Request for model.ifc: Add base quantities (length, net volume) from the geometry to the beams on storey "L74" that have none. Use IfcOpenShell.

First a look at what the model holds.

```python
import ifcopenshell
import ifcopenshell.util.element
import ifcopenshell.util.unit

model = ifcopenshell.open("model.ifc")
print(model.schema)
for unit_type in ("LENGTHUNIT", "AREAUNIT", "VOLUMEUNIT"):
    print(unit_type, ifcopenshell.util.unit.calculate_unit_scale(model, unit_type))
storey = next(s for s in model.by_type("IfcBuildingStorey") if s.Name == "L74")
beams = [e for e in ifcopenshell.util.element.get_decomposition(storey) if e.is_a("IfcBeam")]
for e in sorted(beams, key=lambda e: e.id()):
    print(e.id(), e.is_a(), e.Name, list(ifcopenshell.util.element.get_psets(e, qtos_only=True)), sep=" | ")
```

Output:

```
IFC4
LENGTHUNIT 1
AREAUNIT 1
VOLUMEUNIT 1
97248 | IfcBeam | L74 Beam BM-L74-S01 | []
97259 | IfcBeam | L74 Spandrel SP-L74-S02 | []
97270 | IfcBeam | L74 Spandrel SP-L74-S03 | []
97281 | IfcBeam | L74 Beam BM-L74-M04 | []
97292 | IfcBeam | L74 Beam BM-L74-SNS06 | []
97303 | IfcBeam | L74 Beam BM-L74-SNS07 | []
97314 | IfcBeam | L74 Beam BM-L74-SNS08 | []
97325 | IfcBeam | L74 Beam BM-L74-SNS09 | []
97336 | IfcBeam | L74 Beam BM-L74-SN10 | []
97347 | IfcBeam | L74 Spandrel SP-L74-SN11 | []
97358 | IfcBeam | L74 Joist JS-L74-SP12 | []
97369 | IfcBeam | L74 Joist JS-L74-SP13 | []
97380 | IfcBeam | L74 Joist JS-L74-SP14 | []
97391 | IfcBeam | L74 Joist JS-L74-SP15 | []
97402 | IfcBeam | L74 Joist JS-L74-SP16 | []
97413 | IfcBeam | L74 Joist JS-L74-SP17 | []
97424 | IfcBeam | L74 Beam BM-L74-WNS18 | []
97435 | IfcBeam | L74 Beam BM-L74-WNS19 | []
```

```python
import ifcopenshell
import ifcopenshell.api.pset
import ifcopenshell.geom
import ifcopenshell.util.element
import ifcopenshell.util.shape
import ifcopenshell.util.unit

model = ifcopenshell.open("model.ifc")
unit_scale = ifcopenshell.util.unit.calculate_unit_scale(model)
volume_scale = ifcopenshell.util.unit.calculate_unit_scale(model, "VOLUMEUNIT")
settings = ifcopenshell.geom.settings()

storey = next(s for s in model.by_type("IfcBuildingStorey") if s.Name == "L74")
beams = [e for e in ifcopenshell.util.element.get_decomposition(storey) if e.is_a("IfcBeam")]

for e in sorted(beams, key=lambda e: e.id()):
    if ifcopenshell.util.element.get_psets(e, qtos_only=True, should_inherit=False):
        continue
    # Geometry comes back in metres, in the element's own axes.
    shape = ifcopenshell.geom.create_shape(settings, e)
    values = {
        "Length": ifcopenshell.util.shape.get_max_xyz(shape.geometry) / unit_scale,
        "NetVolume": ifcopenshell.util.shape.get_volume(shape.geometry) / volume_scale,
    }
    qto = ifcopenshell.api.pset.add_qto(model, product=e, name="Qto_BeamBaseQuantities")
    ifcopenshell.api.pset.edit_qto(model, qto=qto, properties=values)
    print(e.id(), {k: round(v, 3) for k, v in values.items()})

model.write("model_rev.ifc")
```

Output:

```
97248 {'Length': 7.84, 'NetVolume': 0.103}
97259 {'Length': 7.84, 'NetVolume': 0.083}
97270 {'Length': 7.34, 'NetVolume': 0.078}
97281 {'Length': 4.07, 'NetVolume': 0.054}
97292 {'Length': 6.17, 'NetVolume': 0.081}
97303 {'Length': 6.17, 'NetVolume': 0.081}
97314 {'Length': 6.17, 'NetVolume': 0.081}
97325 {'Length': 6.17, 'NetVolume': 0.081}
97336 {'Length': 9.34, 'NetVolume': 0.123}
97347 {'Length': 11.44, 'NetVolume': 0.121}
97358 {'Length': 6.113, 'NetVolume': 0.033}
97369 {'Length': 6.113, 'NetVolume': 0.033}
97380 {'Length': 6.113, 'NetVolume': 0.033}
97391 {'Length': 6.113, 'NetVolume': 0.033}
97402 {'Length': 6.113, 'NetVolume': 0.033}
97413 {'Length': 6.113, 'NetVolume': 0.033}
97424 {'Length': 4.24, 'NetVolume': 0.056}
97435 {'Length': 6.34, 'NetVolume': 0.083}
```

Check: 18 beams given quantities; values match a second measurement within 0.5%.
